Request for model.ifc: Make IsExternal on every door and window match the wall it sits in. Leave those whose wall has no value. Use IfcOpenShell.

First a look at what the model holds.

```python
import ifcopenshell
import ifcopenshell.util.element

model = ifcopenshell.open("model.ifc")
print(model.schema)
seen = {}
for e in model.by_type("IfcDoor") + model.by_type("IfcWindow"):
    if not e.FillsVoids:
        continue
    host = e.FillsVoids[0].RelatingOpeningElement.VoidsElements[0].RelatingBuildingElement
    own = ifcopenshell.util.element.get_pset(e, f"Pset_{e.is_a()[3:].removesuffix('StandardCase')}Common", "IsExternal")
    wall = ifcopenshell.util.element.get_pset(host, "Pset_WallCommon", "IsExternal")
    seen[e.is_a(), own, wall] = seen.get((e.is_a(), own, wall), 0) + 1
for (cls, own, wall), count in sorted(seen.items(), key=str):
    print(count, cls, "IsExternal:", own, "| host wall:", wall)
```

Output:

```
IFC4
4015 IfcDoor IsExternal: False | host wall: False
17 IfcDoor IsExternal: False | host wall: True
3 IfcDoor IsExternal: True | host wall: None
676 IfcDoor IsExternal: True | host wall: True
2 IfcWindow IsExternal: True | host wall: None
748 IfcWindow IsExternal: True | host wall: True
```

```python
import ifcopenshell
import ifcopenshell.api.pset
import ifcopenshell.util.element

model = ifcopenshell.open("model.ifc")

count = 0
for ifc_class, pset_name in (("IfcDoor", "Pset_DoorCommon"), ("IfcWindow", "Pset_WindowCommon")):
    for e in model.by_type(ifc_class):
        if not e.FillsVoids:
            continue
        host = e.FillsVoids[0].RelatingOpeningElement.VoidsElements[0].RelatingBuildingElement
        external = ifcopenshell.util.element.get_pset(host, "Pset_WallCommon", "IsExternal")
        if external is None or ifcopenshell.util.element.get_pset(e, pset_name, "IsExternal") == external:
            continue
        found = ifcopenshell.util.element.get_pset(e, pset_name, should_inherit=False)
        if found:
            pset = model.by_id(found["id"])
            if len(ifcopenshell.util.element.get_elements_by_pset(pset)) > 1:
                pset = ifcopenshell.api.pset.unshare_pset(model, products=[e], pset=pset)[0]
        else:
            pset = ifcopenshell.api.pset.add_pset(model, product=e, name=pset_name)
        ifcopenshell.api.pset.edit_pset(model, pset=pset, properties={"IsExternal": external})
        count += 1

print(count, "updated")

model.write("model_v2.ifc")
```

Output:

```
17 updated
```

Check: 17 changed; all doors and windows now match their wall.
